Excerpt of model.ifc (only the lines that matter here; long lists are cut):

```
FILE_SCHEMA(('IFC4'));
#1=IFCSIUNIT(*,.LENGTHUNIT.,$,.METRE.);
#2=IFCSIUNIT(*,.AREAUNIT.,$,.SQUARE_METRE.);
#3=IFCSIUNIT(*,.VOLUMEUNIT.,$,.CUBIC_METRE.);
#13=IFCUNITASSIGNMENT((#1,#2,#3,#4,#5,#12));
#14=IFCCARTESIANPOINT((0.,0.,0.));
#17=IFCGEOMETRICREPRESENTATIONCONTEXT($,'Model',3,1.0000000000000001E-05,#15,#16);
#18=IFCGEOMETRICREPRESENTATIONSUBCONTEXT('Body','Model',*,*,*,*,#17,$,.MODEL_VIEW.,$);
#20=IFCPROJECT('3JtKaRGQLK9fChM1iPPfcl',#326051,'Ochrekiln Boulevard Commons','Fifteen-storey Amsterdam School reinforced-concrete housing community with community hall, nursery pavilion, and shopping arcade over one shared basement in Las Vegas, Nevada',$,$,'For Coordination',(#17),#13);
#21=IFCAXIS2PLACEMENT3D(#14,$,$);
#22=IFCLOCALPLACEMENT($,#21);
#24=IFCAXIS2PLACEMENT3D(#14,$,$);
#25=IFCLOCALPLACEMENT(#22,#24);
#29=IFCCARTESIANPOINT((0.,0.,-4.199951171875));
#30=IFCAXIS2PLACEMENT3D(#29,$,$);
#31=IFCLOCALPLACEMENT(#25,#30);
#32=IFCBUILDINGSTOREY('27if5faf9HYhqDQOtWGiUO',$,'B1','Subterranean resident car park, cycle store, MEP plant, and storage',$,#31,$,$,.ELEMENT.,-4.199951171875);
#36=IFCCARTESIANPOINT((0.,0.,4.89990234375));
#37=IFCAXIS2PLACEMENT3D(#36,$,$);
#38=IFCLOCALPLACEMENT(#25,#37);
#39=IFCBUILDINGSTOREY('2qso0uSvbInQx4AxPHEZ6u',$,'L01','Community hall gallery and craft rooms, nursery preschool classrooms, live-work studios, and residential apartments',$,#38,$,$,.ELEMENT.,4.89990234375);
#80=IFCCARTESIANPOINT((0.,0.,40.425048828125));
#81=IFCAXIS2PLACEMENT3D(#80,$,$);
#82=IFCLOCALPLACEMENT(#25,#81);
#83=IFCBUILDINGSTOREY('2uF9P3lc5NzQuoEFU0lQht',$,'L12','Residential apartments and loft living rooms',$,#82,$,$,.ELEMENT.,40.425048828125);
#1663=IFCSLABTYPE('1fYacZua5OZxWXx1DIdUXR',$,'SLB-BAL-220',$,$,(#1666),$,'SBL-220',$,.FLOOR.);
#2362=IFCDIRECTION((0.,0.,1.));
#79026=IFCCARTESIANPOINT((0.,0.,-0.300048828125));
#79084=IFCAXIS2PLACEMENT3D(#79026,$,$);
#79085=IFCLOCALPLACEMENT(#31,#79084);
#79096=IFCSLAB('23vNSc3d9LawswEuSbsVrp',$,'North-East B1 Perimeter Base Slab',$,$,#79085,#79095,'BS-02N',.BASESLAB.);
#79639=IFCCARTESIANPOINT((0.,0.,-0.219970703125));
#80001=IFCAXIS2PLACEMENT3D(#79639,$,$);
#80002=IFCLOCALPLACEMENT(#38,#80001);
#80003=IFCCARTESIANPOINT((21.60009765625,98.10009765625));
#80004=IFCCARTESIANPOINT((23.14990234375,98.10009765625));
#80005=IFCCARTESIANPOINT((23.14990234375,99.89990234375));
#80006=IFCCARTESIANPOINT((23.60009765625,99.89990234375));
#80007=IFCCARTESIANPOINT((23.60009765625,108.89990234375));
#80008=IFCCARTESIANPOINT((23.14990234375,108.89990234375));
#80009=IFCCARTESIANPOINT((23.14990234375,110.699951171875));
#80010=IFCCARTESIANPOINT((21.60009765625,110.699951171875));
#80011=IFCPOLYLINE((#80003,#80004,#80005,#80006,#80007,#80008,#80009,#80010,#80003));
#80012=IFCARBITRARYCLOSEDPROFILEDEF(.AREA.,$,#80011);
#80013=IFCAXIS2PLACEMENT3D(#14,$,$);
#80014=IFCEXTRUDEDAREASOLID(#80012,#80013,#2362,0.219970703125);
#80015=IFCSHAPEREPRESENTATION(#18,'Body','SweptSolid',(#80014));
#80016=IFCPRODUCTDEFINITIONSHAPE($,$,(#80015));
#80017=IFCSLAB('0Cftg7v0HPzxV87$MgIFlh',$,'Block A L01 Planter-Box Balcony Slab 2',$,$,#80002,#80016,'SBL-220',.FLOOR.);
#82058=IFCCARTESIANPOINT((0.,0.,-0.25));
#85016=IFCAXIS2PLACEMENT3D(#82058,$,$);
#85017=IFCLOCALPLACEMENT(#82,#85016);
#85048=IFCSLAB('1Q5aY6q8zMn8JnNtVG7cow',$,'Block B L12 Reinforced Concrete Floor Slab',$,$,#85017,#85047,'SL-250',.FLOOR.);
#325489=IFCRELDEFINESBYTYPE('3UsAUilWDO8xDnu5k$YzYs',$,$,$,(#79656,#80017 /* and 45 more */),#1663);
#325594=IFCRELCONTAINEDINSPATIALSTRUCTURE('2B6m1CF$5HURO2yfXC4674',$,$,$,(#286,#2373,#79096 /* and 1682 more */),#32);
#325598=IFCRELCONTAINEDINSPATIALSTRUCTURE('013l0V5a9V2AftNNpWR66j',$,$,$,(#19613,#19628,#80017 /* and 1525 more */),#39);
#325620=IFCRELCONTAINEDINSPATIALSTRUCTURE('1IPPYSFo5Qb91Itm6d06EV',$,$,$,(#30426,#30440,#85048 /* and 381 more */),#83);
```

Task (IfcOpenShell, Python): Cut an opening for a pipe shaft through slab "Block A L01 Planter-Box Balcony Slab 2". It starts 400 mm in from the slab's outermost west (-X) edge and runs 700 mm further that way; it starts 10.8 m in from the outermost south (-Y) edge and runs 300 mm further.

```python
import numpy as np
import ifcopenshell
import ifcopenshell.api.feature
import ifcopenshell.api.geometry
import ifcopenshell.api.root
import ifcopenshell.geom
import ifcopenshell.util.placement
import ifcopenshell.util.representation
import ifcopenshell.util.shape
import ifcopenshell.util.unit

model = ifcopenshell.open("model.ifc")
unit_scale = ifcopenshell.util.unit.calculate_unit_scale(model)
settings = ifcopenshell.geom.settings()


def volume(element):
    """Net volume in cubic metres, openings subtracted."""
    shape = ifcopenshell.geom.create_shape(settings, element)
    return ifcopenshell.util.shape.get_volume(shape.geometry)


slab = model.by_guid("0Cftg7v0HPzxV87$MgIFlh")
before = volume(slab)

# Extent in the slab's own axes, in metres. The edges named are its -X and -Y sides.
slab_shape = ifcopenshell.geom.create_shape(settings, slab)
vertices = ifcopenshell.util.shape.get_vertices(slab_shape.geometry)
x_min, y_min, bottom = vertices.min(axis=0)
top = vertices[:, 2].max()

opening = ifcopenshell.api.root.create_entity(model, ifc_class="IfcOpeningElement", name="Pipe shaft opening", predefined_type="OPENING")
context = ifcopenshell.util.representation.get_context(model, "Model", "Body", "MODEL_VIEW")
width, depth = 0.7, 0.3
outline = [(0.0, 0.0), (width, 0.0), (width, depth), (0.0, depth), (0.0, 0.0)]
# Overshoot both faces by 50 mm so the cut is clean.
shape = ifcopenshell.api.geometry.add_slab_representation(
    model, context=context, depth=top - bottom + 0.1, polyline=outline
)
ifcopenshell.api.geometry.assign_representation(model, product=opening, representation=shape)

matrix = ifcopenshell.util.placement.get_local_placement(slab.ObjectPlacement)
matrix[:, 3] = matrix @ np.append(np.array([x_min + 0.4, y_min + 10.8, bottom - 0.05]) / unit_scale, 1.0)
ifcopenshell.api.geometry.edit_object_placement(model, product=opening, matrix=matrix, is_si=False)
ifcopenshell.api.feature.add_feature(model, feature=opening, element=slab)

after = volume(slab)

print(f"slab volume {before:.3f} -> {after:.3f} m3")

model.write("model_edited.ifc")
```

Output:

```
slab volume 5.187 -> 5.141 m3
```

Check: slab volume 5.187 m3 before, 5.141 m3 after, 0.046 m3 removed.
